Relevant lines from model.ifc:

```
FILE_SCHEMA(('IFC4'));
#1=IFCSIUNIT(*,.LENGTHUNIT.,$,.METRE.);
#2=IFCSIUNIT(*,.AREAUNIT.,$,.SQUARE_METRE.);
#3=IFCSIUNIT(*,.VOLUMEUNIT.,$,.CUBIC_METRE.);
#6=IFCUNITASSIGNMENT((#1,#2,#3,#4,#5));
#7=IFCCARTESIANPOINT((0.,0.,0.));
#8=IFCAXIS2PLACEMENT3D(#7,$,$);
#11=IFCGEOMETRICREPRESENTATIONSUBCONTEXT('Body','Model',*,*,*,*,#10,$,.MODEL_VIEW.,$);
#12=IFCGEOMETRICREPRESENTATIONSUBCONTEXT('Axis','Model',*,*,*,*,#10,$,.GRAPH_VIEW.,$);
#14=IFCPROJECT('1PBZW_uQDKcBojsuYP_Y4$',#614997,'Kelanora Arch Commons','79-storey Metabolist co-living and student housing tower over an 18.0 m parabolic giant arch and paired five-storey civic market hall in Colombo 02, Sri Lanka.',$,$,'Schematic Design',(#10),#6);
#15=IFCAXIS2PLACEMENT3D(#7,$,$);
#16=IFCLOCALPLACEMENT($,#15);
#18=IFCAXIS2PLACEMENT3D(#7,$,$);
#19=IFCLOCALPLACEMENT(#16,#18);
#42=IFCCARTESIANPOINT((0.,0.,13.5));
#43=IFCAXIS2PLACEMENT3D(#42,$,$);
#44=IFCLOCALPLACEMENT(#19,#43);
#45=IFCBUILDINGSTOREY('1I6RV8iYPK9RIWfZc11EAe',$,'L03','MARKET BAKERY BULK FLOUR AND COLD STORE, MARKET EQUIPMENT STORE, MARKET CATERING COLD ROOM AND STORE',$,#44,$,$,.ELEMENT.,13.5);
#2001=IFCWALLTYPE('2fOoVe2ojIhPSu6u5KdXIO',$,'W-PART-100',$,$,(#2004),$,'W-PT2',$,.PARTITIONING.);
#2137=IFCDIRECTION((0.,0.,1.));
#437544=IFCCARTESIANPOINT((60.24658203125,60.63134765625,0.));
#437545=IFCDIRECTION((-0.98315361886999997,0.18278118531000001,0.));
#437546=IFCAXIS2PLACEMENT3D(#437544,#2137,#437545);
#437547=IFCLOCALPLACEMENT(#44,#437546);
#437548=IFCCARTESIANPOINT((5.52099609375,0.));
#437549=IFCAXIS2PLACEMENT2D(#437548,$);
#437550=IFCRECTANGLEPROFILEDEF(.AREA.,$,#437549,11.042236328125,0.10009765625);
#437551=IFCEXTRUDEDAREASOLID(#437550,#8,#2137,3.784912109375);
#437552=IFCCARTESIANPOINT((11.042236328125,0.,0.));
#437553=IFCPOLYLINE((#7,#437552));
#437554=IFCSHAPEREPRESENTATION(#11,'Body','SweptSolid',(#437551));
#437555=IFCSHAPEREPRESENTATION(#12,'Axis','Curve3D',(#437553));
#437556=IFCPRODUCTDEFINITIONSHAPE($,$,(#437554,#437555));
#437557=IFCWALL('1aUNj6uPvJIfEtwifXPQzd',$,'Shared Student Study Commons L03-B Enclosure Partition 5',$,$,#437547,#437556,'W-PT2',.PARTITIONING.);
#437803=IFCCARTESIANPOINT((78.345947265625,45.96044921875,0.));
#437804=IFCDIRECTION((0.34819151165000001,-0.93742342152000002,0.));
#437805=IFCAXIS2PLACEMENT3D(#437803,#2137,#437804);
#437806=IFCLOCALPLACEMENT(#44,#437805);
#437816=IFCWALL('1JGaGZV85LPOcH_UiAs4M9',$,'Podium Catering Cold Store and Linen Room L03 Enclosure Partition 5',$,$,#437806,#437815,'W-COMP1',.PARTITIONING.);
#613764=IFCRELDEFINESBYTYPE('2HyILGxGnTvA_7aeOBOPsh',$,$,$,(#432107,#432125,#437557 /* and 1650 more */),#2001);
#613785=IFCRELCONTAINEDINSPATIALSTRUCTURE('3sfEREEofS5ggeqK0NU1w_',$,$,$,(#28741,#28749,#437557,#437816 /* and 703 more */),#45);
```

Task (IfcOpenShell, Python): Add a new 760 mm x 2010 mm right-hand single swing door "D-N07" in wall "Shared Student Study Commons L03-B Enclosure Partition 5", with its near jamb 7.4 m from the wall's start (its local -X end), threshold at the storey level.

```python
import numpy as np
import ifcopenshell
import ifcopenshell.api.feature
import ifcopenshell.api.geometry
import ifcopenshell.api.root
import ifcopenshell.api.spatial
import ifcopenshell.geom
import ifcopenshell.util.element
import ifcopenshell.util.placement
import ifcopenshell.util.representation
import ifcopenshell.util.shape
import ifcopenshell.util.unit

model = ifcopenshell.open("model.ifc")
unit_scale = ifcopenshell.util.unit.calculate_unit_scale(model)
settings = ifcopenshell.geom.settings()


def volume(element):
    """Net volume in cubic metres, openings subtracted."""
    shape = ifcopenshell.geom.create_shape(settings, element)
    return ifcopenshell.util.shape.get_volume(shape.geometry)


wall = model.by_guid("1aUNj6uPvJIfEtwifXPQzd")
storey = ifcopenshell.util.element.get_container(wall, ifc_class="IfcBuildingStorey")
context = ifcopenshell.util.representation.get_context(model, "Model", "Body", "MODEL_VIEW")
before = volume(wall)

width, height, from_end, sill = 0.76, 2.01, 7.4, 0.0  # metres

# The wall runs along its own X axis, and the end named is its -X end.
wall_shape = ifcopenshell.geom.create_shape(settings, wall)
x, y, z = ifcopenshell.util.shape.get_vertices(wall_shape.geometry).T
start = x.min() + from_end
face, thickness = float(y.min()), float(y.max() - y.min())
wall_matrix = ifcopenshell.util.placement.get_local_placement(wall.ObjectPlacement)
level = ifcopenshell.util.placement.get_local_placement(storey.ObjectPlacement)[2, 3]


def in_wall(x, y):
    """Placement at x, y metres in the wall's axes, at sill height."""
    matrix = wall_matrix.copy()
    matrix[:, 3] = wall_matrix @ np.array([x / unit_scale, y / unit_scale, 0.0, 1.0])
    matrix[2, 3] = level + sill / unit_scale
    return matrix


# Opening: a box that overshoots both wall faces by 50 mm.
opening = ifcopenshell.api.root.create_entity(model, ifc_class="IfcOpeningElement", predefined_type="OPENING")
box = ifcopenshell.api.geometry.add_wall_representation(
    model, context=context, length=width, height=height, thickness=thickness + 0.1
)
ifcopenshell.api.geometry.assign_representation(model, product=opening, representation=box)
ifcopenshell.api.geometry.edit_object_placement(model, product=opening, matrix=in_wall(start, face - 0.05), is_si=False)
ifcopenshell.api.feature.add_feature(model, feature=opening, element=wall)

door = ifcopenshell.api.root.create_entity(model, ifc_class="IfcDoor", name="D-N07", predefined_type="DOOR")
door.OverallWidth, door.OverallHeight = width / unit_scale, height / unit_scale
door.OperationType = "SINGLE_SWING_RIGHT"
body = ifcopenshell.api.geometry.add_door_representation(
    model,
    context=context,
    overall_width=door.OverallWidth,
    overall_height=door.OverallHeight,
    operation_type="SINGLE_SWING_RIGHT",
    lining_properties={"LiningDepth": thickness / unit_scale, "ThresholdDepth": thickness / unit_scale},
)
ifcopenshell.api.geometry.assign_representation(model, product=door, representation=body)
ifcopenshell.api.spatial.assign_container(model, products=[door], relating_structure=storey)
ifcopenshell.api.feature.add_filling(model, opening=opening, element=door)

# The lining spans the wall, so the door starts at the wall face.
ifcopenshell.api.geometry.edit_object_placement(model, product=door, matrix=in_wall(start, face), is_si=False)

after = volume(wall)

print(f"wall volume {before:.3f} -> {after:.3f} m3")

model.write("model_edited.ifc")
```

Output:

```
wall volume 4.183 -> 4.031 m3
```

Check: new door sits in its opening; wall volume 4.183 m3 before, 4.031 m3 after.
